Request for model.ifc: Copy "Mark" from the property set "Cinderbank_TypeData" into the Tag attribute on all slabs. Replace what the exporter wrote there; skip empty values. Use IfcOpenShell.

First a look at what the model holds.

```python
import ifcopenshell
import ifcopenshell.util.element

model = ifcopenshell.open("model.ifc")
print(model.schema)
slabs = model.by_type("IfcSlab")
print(len(slabs), "slabs")
for e in slabs[:8]:
    source = ifcopenshell.util.element.get_pset(e, "Cinderbank_TypeData", "Mark")
    target = e.Tag
    print(e.id(), repr(source), repr(target), sep=" | ")
```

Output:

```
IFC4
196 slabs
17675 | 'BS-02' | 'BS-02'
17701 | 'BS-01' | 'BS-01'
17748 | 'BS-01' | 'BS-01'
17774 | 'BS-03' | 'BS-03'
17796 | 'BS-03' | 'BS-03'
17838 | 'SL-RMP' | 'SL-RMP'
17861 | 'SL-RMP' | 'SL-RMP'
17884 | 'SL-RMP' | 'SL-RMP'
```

```python
import ifcopenshell
import ifcopenshell.util.element

model = ifcopenshell.open("model.ifc")

count = 0
for e in model.by_type("IfcSlab"):
    value = ifcopenshell.util.element.get_pset(e, "Cinderbank_TypeData", "Mark")
    current = e.Tag
    if not value or not value.strip() or current == value:
        continue
    e.Tag = value
    count += 1

print(count, "slabs updated")

model.write("model_updated.ifc")
```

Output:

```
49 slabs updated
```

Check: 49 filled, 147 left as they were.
